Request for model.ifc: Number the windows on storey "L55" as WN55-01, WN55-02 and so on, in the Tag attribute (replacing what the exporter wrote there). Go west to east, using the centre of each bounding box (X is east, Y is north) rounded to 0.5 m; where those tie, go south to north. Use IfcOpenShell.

First a look at what the model holds.

```python
import ifcopenshell
import ifcopenshell.util.element
import ifcopenshell.util.placement

model = ifcopenshell.open("model.ifc")
print(model.schema)
storey = next(s for s in model.by_type("IfcBuildingStorey") if s.Name == "L55")
windows = [e for e in ifcopenshell.util.element.get_decomposition(storey) if e.is_a("IfcWindow")]
for e in sorted(windows, key=lambda e: e.id()):
    origin = ifcopenshell.util.placement.get_local_placement(e.ObjectPlacement)[:3, 3]
    print(e.id(), e.Tag, e.Name, origin.round(2) + 0.0, sep=" | ")
```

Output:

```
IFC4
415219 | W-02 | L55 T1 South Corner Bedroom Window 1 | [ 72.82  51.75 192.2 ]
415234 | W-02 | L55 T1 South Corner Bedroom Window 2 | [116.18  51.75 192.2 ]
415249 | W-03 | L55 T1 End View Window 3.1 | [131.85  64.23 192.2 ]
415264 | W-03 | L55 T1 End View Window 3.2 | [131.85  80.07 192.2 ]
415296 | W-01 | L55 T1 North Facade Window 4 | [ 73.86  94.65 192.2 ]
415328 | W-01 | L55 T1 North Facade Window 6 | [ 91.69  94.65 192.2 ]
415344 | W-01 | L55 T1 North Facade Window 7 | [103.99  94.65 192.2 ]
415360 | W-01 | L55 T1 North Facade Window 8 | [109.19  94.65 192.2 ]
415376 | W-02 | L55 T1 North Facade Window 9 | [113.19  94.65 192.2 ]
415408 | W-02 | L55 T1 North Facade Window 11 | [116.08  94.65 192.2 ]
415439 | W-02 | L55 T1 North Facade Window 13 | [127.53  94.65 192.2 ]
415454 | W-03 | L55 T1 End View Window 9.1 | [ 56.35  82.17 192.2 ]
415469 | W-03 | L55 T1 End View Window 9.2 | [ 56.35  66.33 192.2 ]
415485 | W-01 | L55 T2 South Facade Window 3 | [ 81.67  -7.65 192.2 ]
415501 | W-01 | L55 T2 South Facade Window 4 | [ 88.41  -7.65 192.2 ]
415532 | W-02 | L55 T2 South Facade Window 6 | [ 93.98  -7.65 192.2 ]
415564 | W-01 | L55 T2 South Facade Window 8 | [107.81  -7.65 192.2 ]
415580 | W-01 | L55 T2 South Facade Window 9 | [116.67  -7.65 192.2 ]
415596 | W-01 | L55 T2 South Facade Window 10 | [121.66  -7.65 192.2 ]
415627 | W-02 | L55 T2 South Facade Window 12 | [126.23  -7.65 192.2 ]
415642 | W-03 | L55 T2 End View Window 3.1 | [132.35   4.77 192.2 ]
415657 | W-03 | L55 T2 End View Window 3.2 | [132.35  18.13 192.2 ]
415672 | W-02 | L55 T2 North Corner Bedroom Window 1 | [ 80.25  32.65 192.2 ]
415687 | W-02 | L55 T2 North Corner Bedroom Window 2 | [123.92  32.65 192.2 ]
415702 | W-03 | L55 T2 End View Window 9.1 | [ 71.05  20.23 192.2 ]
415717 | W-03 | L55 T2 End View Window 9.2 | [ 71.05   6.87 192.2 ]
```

```python
import ifcopenshell
import ifcopenshell.geom
import ifcopenshell.util.element
import ifcopenshell.util.shape

model = ifcopenshell.open("model.ifc")
settings = ifcopenshell.geom.settings()
settings.set("use-world-coords", True)


def centre(element):
    shape = ifcopenshell.geom.create_shape(settings, element)
    return ifcopenshell.util.shape.get_bbox_centroid(shape.geometry)


storey = next(s for s in model.by_type("IfcBuildingStorey") if s.Name == "L55")
windows = [e for e in ifcopenshell.util.element.get_decomposition(storey) if e.is_a("IfcWindow")]

# Insertion points can sit at a corner or the storey origin, so sort by the geometry (in metres).
centres = {e: centre(e) for e in windows}
windows.sort(key=lambda e: (round(centres[e][0] / 0.5), centres[e][1]))

for i, e in enumerate(windows, start=1):
    number = f"WN55-{i:02d}"
    e.Tag = number
    print(e.id(), number)

model.write("model_edited.ifc")
```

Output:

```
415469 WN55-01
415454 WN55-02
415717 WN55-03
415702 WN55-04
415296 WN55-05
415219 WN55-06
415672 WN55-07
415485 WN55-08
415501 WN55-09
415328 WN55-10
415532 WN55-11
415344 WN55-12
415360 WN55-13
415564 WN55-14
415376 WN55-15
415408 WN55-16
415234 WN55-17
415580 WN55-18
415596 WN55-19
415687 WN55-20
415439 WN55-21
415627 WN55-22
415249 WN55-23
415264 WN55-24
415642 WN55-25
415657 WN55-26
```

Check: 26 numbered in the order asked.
